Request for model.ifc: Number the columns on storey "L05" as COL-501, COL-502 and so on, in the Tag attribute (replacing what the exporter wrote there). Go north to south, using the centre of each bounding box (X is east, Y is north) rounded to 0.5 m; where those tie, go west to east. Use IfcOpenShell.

First a look at what the model holds.

```python
import ifcopenshell
import ifcopenshell.util.element
import ifcopenshell.util.placement

model = ifcopenshell.open("model.ifc")
print(model.schema)
storey = next(s for s in model.by_type("IfcBuildingStorey") if s.Name == "L05")
columns = [e for e in ifcopenshell.util.element.get_decomposition(storey) if e.is_a("IfcColumn")]
for e in sorted(columns, key=lambda e: e.id()):
    origin = ifcopenshell.util.placement.get_local_placement(e.ObjectPlacement)[:3, 3]
    print(e.id(), e.Tag, e.Name, origin.round(2) + 0.0, sep=" | ")
```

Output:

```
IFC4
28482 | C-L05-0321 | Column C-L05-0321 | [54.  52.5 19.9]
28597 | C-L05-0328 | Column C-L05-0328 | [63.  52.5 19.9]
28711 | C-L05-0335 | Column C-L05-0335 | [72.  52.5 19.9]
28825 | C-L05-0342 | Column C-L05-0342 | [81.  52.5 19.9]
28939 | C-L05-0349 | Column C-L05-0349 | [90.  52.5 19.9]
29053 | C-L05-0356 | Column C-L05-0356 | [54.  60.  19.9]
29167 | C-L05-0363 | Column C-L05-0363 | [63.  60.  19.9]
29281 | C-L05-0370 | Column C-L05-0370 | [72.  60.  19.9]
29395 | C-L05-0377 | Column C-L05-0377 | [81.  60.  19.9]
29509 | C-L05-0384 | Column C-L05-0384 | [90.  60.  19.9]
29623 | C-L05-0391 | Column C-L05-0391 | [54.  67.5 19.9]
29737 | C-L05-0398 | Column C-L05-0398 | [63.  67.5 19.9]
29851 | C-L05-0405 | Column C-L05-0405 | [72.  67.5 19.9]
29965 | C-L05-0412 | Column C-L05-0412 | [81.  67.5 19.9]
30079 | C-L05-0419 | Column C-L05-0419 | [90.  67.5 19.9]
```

```python
import ifcopenshell
import ifcopenshell.geom
import ifcopenshell.util.element
import ifcopenshell.util.shape

model = ifcopenshell.open("model.ifc")
settings = ifcopenshell.geom.settings()
settings.set("use-world-coords", True)


def centre(element):
    shape = ifcopenshell.geom.create_shape(settings, element)
    return ifcopenshell.util.shape.get_bbox_centroid(shape.geometry)


storey = next(s for s in model.by_type("IfcBuildingStorey") if s.Name == "L05")
columns = [e for e in ifcopenshell.util.element.get_decomposition(storey) if e.is_a("IfcColumn")]

# Insertion points can sit at a corner or the storey origin, so sort by the geometry (in metres).
centres = {e: centre(e) for e in columns}
columns.sort(key=lambda e: (-round(centres[e][1] / 0.5), centres[e][0]))

for i, e in enumerate(columns, start=1):
    number = f"COL-5{i:02d}"
    e.Tag = number
    print(e.id(), number)

model.write("model_v2.ifc")
```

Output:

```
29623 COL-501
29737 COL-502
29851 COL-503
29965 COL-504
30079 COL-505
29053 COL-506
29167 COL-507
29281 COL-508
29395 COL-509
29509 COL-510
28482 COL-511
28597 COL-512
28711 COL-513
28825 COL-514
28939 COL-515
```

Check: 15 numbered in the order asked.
